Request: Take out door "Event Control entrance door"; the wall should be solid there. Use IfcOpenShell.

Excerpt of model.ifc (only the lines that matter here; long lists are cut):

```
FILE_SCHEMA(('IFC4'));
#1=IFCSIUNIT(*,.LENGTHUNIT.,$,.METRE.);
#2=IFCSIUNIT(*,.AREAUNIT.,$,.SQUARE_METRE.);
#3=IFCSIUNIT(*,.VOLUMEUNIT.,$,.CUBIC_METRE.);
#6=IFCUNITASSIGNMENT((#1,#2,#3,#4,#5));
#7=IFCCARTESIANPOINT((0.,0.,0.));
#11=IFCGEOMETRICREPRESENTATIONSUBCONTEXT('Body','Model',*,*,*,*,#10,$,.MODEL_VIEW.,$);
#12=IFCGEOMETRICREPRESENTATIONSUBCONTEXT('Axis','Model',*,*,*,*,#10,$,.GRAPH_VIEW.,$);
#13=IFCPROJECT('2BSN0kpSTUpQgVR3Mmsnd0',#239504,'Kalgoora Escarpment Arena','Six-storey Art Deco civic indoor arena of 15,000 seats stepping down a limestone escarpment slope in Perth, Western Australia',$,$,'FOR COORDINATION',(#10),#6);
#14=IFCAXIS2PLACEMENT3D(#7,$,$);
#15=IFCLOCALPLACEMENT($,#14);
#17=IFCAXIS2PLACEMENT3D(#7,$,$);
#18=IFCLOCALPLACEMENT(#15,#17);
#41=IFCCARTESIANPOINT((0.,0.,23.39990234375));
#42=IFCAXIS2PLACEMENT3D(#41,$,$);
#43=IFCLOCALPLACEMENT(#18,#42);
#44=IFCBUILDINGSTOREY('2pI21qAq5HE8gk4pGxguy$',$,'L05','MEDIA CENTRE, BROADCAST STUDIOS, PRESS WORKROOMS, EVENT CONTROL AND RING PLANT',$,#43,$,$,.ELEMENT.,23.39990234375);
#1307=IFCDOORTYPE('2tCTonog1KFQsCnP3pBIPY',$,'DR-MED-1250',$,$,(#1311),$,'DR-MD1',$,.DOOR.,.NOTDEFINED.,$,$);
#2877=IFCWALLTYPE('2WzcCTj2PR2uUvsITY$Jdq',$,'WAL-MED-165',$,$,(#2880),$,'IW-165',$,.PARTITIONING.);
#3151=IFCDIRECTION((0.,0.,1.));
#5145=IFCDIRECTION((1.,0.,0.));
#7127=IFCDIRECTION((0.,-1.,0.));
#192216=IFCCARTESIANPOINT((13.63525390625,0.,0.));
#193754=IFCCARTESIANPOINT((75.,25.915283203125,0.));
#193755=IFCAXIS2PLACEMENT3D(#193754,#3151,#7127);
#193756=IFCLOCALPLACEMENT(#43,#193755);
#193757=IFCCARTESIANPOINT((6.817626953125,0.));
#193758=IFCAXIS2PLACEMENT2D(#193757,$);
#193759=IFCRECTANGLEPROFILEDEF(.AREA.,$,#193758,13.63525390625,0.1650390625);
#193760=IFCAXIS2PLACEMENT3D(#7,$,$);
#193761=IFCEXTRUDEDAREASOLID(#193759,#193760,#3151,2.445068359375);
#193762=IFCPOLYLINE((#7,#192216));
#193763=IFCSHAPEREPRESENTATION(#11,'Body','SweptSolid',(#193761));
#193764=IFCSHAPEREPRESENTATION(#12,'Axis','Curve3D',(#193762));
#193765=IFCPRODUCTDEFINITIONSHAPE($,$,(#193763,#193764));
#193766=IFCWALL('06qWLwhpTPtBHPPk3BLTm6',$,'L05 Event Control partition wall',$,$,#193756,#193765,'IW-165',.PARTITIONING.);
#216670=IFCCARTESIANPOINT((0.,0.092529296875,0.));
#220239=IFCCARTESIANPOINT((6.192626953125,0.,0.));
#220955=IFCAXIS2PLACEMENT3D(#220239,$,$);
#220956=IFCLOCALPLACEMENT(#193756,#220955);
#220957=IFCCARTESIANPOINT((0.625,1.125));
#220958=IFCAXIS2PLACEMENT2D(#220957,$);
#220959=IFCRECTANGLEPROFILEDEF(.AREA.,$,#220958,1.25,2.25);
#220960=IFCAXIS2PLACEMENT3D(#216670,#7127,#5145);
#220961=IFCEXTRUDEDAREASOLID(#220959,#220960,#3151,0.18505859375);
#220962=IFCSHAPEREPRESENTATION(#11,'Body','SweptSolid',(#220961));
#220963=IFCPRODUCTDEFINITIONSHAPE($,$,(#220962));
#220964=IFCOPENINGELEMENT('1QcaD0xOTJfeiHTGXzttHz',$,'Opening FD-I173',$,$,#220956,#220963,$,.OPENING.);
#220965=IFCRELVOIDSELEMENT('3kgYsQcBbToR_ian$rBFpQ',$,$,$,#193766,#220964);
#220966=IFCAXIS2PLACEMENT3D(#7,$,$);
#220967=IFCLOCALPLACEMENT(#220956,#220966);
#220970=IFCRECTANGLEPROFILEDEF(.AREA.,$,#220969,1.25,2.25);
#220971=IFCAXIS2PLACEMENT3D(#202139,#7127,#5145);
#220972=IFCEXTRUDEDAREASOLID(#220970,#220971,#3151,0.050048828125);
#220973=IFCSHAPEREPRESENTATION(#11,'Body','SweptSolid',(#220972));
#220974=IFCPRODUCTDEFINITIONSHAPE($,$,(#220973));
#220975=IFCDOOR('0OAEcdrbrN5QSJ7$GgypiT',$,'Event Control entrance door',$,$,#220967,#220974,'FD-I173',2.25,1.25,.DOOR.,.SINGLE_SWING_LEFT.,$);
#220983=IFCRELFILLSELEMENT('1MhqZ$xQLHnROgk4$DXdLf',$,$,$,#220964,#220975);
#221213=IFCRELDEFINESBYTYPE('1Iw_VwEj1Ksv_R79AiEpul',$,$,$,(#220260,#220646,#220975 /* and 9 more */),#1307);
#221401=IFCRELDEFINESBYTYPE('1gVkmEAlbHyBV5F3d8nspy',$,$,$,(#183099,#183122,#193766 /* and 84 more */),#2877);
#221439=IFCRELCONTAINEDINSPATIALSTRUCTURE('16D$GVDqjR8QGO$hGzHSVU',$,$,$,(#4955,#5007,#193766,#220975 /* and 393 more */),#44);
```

```python
import ifcopenshell
import ifcopenshell.api.feature
import ifcopenshell.api.root
import ifcopenshell.geom
import ifcopenshell.util.shape

model = ifcopenshell.open("model.ifc")
settings = ifcopenshell.geom.settings()


def volume(element):
    """Net volume in cubic metres, openings subtracted."""
    shape = ifcopenshell.geom.create_shape(settings, element)
    return ifcopenshell.util.shape.get_volume(shape.geometry)


door = model.by_guid("0OAEcdrbrN5QSJ7$GgypiT")
opening = door.FillsVoids[0].RelatingOpeningElement
wall = opening.VoidsElements[0].RelatingBuildingElement
before = volume(wall)

ifcopenshell.api.root.remove_product(model, product=door)
ifcopenshell.api.feature.remove_feature(model, feature=opening)

after = volume(wall)

print(f"wall volume {before:.3f} -> {after:.3f} m3")

model.write("model_edited.ifc")
```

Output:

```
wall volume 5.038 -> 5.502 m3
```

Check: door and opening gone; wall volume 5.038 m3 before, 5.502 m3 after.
